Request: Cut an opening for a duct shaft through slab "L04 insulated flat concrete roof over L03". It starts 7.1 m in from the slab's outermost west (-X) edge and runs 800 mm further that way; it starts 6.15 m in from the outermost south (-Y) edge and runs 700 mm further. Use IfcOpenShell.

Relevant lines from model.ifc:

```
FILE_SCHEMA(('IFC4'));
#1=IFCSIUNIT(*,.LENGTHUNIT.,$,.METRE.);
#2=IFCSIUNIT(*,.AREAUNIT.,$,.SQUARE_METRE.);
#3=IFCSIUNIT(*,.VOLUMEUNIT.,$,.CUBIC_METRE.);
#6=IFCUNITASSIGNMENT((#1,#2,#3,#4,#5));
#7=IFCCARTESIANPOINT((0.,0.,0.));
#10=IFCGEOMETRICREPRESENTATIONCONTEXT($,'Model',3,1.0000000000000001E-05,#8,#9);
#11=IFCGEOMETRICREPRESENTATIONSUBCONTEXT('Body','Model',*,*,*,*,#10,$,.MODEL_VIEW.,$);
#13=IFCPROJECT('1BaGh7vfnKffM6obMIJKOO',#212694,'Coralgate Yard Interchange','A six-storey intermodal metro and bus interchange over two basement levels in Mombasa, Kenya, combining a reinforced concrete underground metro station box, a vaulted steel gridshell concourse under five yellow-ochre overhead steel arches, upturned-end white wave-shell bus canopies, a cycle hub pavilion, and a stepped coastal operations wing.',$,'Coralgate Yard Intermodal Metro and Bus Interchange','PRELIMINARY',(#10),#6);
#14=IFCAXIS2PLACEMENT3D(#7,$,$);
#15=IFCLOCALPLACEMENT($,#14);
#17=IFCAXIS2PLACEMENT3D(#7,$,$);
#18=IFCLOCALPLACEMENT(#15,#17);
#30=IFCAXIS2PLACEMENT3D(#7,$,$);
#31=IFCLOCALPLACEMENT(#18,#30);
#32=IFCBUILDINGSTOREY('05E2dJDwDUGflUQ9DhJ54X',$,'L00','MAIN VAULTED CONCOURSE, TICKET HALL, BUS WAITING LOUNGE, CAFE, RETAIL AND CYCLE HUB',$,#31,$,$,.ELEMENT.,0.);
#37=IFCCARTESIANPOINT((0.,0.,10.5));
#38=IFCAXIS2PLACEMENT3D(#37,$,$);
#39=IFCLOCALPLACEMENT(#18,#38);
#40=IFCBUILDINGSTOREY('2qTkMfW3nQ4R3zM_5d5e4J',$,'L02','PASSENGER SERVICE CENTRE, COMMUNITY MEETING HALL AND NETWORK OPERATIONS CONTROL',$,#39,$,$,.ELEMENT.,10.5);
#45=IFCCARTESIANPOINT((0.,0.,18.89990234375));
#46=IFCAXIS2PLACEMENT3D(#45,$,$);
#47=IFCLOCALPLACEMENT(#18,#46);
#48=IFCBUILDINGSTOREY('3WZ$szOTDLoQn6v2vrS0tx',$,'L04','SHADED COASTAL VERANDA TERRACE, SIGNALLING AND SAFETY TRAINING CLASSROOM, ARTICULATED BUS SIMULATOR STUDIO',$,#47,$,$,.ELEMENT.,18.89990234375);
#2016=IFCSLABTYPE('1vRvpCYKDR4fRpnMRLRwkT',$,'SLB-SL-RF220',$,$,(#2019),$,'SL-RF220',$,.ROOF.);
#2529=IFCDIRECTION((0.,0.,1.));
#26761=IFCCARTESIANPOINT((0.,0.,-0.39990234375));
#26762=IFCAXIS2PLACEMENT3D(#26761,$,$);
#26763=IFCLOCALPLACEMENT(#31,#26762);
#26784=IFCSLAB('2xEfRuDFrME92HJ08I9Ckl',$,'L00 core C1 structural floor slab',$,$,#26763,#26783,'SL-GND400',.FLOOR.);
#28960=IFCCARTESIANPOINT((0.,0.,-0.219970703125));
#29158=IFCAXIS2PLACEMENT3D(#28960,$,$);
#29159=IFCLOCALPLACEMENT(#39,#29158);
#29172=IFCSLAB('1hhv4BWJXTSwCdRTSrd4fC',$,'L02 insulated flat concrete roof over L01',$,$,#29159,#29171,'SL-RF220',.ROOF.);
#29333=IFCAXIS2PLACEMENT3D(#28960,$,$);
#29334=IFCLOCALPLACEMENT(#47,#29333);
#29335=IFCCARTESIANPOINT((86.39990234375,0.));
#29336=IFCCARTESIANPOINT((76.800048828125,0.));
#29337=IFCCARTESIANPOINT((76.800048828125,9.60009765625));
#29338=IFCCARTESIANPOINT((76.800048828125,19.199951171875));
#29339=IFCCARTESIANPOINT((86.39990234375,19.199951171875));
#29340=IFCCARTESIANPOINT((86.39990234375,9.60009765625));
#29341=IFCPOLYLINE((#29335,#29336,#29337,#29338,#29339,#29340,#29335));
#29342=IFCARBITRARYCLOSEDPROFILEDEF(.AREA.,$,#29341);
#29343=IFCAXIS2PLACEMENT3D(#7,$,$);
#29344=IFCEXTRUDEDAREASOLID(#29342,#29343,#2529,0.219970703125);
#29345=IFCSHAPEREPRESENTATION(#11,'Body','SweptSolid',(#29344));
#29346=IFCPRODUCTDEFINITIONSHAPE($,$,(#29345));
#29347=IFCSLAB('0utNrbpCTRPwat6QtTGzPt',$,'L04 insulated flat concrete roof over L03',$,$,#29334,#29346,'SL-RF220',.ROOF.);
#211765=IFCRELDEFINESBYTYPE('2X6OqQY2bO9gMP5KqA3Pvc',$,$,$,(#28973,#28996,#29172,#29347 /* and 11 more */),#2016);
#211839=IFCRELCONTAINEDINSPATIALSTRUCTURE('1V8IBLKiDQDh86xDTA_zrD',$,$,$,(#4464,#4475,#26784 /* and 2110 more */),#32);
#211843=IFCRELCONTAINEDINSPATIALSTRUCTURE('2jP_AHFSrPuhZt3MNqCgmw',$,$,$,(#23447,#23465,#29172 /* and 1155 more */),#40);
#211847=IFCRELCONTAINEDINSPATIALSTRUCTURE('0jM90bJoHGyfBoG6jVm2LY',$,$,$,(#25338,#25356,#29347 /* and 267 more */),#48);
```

```python
import numpy as np
import ifcopenshell
import ifcopenshell.api.feature
import ifcopenshell.api.geometry
import ifcopenshell.api.root
import ifcopenshell.geom
import ifcopenshell.util.placement
import ifcopenshell.util.representation
import ifcopenshell.util.shape
import ifcopenshell.util.unit

model = ifcopenshell.open("model.ifc")
unit_scale = ifcopenshell.util.unit.calculate_unit_scale(model)
settings = ifcopenshell.geom.settings()


def volume(element):
    """Net volume in cubic metres, openings subtracted."""
    shape = ifcopenshell.geom.create_shape(settings, element)
    return ifcopenshell.util.shape.get_volume(shape.geometry)


slab = model.by_guid("0utNrbpCTRPwat6QtTGzPt")
before = volume(slab)

# Extent in the slab's own axes, in metres. The edges named are its -X and -Y sides.
slab_shape = ifcopenshell.geom.create_shape(settings, slab)
vertices = ifcopenshell.util.shape.get_vertices(slab_shape.geometry)
x_min, y_min, bottom = vertices.min(axis=0)
top = vertices[:, 2].max()

opening = ifcopenshell.api.root.create_entity(model, ifc_class="IfcOpeningElement", name="Duct shaft opening", predefined_type="OPENING")
context = ifcopenshell.util.representation.get_context(model, "Model", "Body", "MODEL_VIEW")
width, depth = 0.8, 0.7
outline = [(0.0, 0.0), (width, 0.0), (width, depth), (0.0, depth), (0.0, 0.0)]
# Overshoot both faces by 50 mm so the cut is clean.
shape = ifcopenshell.api.geometry.add_slab_representation(
    model, context=context, depth=top - bottom + 0.1, polyline=outline
)
ifcopenshell.api.geometry.assign_representation(model, product=opening, representation=shape)

matrix = ifcopenshell.util.placement.get_local_placement(slab.ObjectPlacement)
matrix[:, 3] = matrix @ np.append(np.array([x_min + 7.1, y_min + 6.15, bottom - 0.05]) / unit_scale, 1.0)
ifcopenshell.api.geometry.edit_object_placement(model, product=opening, matrix=matrix, is_si=False)
ifcopenshell.api.feature.add_feature(model, feature=opening, element=slab)

after = volume(slab)

print(f"slab volume {before:.3f} -> {after:.3f} m3")

model.write("model_edited.ifc")
```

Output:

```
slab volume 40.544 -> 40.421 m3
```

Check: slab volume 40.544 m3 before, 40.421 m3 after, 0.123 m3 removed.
